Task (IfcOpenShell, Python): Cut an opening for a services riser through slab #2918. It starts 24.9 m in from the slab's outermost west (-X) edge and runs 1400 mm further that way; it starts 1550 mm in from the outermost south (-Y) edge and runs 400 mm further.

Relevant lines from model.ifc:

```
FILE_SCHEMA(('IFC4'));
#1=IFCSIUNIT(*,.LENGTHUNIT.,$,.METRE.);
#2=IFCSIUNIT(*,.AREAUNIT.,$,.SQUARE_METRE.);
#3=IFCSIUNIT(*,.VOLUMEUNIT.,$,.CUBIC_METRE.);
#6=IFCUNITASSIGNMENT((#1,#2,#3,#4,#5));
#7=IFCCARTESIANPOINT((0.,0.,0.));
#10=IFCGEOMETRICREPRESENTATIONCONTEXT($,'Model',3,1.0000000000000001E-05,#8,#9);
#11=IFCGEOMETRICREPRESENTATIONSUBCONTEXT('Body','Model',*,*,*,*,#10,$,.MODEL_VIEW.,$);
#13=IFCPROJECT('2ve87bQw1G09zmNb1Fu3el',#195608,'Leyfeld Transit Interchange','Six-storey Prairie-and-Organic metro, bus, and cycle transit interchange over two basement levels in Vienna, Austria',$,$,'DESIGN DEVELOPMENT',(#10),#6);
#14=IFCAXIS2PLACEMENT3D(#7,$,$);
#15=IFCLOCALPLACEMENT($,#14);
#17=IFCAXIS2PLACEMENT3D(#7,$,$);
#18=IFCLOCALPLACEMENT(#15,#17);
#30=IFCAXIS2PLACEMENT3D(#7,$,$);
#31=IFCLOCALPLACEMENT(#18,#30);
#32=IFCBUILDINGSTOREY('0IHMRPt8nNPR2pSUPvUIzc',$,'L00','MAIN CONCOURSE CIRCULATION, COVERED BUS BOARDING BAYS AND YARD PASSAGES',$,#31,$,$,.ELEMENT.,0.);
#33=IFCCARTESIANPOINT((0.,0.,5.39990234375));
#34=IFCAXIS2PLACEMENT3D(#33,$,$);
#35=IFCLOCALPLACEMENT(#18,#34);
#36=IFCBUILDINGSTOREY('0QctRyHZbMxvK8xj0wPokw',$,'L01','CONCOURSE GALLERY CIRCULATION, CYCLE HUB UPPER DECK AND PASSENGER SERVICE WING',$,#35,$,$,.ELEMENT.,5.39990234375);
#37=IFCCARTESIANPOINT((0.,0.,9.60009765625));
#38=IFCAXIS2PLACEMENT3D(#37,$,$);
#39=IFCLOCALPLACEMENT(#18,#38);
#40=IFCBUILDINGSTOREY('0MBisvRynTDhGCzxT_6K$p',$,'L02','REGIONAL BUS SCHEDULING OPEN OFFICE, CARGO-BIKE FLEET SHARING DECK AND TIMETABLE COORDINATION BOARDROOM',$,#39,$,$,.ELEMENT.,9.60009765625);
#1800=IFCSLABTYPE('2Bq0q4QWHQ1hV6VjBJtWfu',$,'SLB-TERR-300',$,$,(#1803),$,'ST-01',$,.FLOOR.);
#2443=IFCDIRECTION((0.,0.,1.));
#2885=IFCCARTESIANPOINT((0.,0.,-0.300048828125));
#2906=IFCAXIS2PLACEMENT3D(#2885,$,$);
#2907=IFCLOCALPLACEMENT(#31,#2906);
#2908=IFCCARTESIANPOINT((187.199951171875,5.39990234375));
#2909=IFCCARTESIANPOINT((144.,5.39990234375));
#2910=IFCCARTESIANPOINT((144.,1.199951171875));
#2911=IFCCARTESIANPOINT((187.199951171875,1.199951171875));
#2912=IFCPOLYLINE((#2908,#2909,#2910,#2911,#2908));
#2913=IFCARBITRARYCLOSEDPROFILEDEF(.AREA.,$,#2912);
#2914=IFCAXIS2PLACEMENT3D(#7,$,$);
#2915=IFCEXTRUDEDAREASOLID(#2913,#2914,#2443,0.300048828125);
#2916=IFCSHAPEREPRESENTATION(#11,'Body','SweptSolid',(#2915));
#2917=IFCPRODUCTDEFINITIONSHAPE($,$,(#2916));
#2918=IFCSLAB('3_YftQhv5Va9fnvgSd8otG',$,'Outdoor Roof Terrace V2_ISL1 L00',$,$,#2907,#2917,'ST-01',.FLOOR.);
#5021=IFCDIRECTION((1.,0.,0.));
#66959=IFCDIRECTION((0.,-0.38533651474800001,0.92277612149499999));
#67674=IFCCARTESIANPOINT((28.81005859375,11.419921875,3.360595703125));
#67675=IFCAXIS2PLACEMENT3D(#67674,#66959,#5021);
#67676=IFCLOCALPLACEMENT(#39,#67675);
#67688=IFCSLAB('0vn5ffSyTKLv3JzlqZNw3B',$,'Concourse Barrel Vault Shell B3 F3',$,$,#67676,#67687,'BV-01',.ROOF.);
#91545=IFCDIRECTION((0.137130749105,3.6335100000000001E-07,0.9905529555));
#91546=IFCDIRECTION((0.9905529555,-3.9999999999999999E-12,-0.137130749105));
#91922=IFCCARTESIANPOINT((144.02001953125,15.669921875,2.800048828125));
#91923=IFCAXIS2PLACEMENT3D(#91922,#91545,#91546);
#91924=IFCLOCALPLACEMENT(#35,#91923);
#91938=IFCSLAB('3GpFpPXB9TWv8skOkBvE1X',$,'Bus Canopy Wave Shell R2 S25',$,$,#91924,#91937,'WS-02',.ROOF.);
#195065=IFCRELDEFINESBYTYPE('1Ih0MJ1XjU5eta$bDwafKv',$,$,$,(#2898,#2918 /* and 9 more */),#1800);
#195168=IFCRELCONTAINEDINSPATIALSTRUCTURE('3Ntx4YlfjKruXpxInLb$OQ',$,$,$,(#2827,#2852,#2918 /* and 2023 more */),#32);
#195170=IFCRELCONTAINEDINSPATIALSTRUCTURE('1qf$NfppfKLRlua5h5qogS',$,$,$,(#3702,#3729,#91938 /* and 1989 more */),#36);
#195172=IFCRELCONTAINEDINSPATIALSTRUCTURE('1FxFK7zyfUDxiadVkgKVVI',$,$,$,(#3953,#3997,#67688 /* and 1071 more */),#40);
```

```python
import numpy as np
import ifcopenshell
import ifcopenshell.api.feature
import ifcopenshell.api.geometry
import ifcopenshell.api.root
import ifcopenshell.geom
import ifcopenshell.util.placement
import ifcopenshell.util.representation
import ifcopenshell.util.shape
import ifcopenshell.util.unit

model = ifcopenshell.open("model.ifc")
unit_scale = ifcopenshell.util.unit.calculate_unit_scale(model)
settings = ifcopenshell.geom.settings()


def volume(element):
    """Net volume in cubic metres, openings subtracted."""
    shape = ifcopenshell.geom.create_shape(settings, element)
    return ifcopenshell.util.shape.get_volume(shape.geometry)


slab = model.by_id(2918)
before = volume(slab)

# Extent in the slab's own axes, in metres. The edges named are its -X and -Y sides.
slab_shape = ifcopenshell.geom.create_shape(settings, slab)
vertices = ifcopenshell.util.shape.get_vertices(slab_shape.geometry)
x_min, y_min, bottom = vertices.min(axis=0)
top = vertices[:, 2].max()

opening = ifcopenshell.api.root.create_entity(model, ifc_class="IfcOpeningElement", name="Services riser opening", predefined_type="OPENING")
context = ifcopenshell.util.representation.get_context(model, "Model", "Body", "MODEL_VIEW")
width, depth = 1.4, 0.4
outline = [(0.0, 0.0), (width, 0.0), (width, depth), (0.0, depth), (0.0, 0.0)]
# Overshoot both faces by 50 mm so the cut is clean.
shape = ifcopenshell.api.geometry.add_slab_representation(
    model, context=context, depth=top - bottom + 0.1, polyline=outline
)
ifcopenshell.api.geometry.assign_representation(model, product=opening, representation=shape)

matrix = ifcopenshell.util.placement.get_local_placement(slab.ObjectPlacement)
matrix[:, 3] = matrix @ np.append(np.array([x_min + 24.9, y_min + 1.55, bottom - 0.05]) / unit_scale, 1.0)
ifcopenshell.api.geometry.edit_object_placement(model, product=opening, matrix=matrix, is_si=False)
ifcopenshell.api.feature.add_feature(model, feature=opening, element=slab)

after = volume(slab)

print(f"slab volume {before:.3f} -> {after:.3f} m3")

model.write("model_rev.ifc")
```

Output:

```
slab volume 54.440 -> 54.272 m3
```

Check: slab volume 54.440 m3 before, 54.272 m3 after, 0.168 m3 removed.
